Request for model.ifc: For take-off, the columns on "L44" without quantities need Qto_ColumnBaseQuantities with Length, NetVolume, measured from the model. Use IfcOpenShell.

First a look at what the model holds.

```python
import ifcopenshell
import ifcopenshell.util.element
import ifcopenshell.util.unit

model = ifcopenshell.open("model.ifc")
print(model.schema)
for unit_type in ("LENGTHUNIT", "AREAUNIT", "VOLUMEUNIT"):
    print(unit_type, ifcopenshell.util.unit.calculate_unit_scale(model, unit_type))
storey = next(s for s in model.by_type("IfcBuildingStorey") if s.Name == "L44")
columns = [e for e in ifcopenshell.util.element.get_decomposition(storey) if e.is_a("IfcColumn")]
for e in sorted(columns, key=lambda e: e.id()):
    print(e.id(), e.is_a(), e.Name, list(ifcopenshell.util.element.get_psets(e, qtos_only=True)), sep=" | ")
```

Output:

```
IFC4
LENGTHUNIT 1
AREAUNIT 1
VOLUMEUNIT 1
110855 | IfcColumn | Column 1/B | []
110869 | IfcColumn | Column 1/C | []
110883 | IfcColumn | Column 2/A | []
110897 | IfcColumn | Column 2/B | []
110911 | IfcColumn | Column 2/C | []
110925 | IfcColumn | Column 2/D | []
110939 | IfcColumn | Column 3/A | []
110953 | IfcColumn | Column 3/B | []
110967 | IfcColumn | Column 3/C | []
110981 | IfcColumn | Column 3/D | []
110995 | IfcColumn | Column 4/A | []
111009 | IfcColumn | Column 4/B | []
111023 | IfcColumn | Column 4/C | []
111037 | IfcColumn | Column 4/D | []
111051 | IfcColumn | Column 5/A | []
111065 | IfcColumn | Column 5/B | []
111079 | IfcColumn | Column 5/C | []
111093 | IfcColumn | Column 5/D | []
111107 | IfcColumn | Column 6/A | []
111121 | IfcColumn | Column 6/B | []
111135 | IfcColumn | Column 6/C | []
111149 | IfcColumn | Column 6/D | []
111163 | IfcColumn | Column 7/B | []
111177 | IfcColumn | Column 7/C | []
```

```python
import ifcopenshell
import ifcopenshell.api.pset
import ifcopenshell.geom
import ifcopenshell.util.element
import ifcopenshell.util.shape
import ifcopenshell.util.unit

model = ifcopenshell.open("model.ifc")
unit_scale = ifcopenshell.util.unit.calculate_unit_scale(model)
volume_scale = ifcopenshell.util.unit.calculate_unit_scale(model, "VOLUMEUNIT")
settings = ifcopenshell.geom.settings()

storey = next(s for s in model.by_type("IfcBuildingStorey") if s.Name == "L44")
columns = [e for e in ifcopenshell.util.element.get_decomposition(storey) if e.is_a("IfcColumn")]

for e in sorted(columns, key=lambda e: e.id()):
    if ifcopenshell.util.element.get_psets(e, qtos_only=True, should_inherit=False):
        continue
    # Geometry comes back in metres, in the element's own axes.
    shape = ifcopenshell.geom.create_shape(settings, e)
    values = {
        "Length": ifcopenshell.util.shape.get_z(shape.geometry) / unit_scale,
        "NetVolume": ifcopenshell.util.shape.get_volume(shape.geometry) / volume_scale,
    }
    qto = ifcopenshell.api.pset.add_qto(model, product=e, name="Qto_ColumnBaseQuantities")
    ifcopenshell.api.pset.edit_qto(model, qto=qto, properties=values)
    print(e.id(), {k: round(v, 3) for k, v in values.items()})

model.write("model_updated.ifc")
```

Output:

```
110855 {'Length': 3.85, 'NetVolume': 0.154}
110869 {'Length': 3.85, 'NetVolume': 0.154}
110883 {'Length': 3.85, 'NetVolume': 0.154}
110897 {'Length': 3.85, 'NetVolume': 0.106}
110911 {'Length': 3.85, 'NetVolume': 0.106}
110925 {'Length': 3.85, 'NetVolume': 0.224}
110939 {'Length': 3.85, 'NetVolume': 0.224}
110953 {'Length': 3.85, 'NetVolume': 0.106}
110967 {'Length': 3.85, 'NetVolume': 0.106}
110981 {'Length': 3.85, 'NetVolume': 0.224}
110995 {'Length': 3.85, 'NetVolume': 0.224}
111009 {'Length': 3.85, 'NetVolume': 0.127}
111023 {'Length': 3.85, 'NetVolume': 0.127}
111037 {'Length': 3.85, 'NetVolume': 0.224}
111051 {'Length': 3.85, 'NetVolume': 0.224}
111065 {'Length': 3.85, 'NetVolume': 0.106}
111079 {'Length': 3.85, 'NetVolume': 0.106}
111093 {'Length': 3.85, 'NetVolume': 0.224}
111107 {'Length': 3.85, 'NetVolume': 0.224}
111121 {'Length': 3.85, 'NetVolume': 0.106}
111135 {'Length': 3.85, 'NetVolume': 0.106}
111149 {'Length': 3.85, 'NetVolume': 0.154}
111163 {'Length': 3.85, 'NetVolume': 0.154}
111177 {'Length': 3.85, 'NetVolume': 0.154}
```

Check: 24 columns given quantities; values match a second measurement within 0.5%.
